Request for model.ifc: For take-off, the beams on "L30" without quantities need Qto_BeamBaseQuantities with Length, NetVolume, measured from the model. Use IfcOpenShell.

First a look at what the model holds.

```python
import ifcopenshell
import ifcopenshell.util.element
import ifcopenshell.util.unit

model = ifcopenshell.open("model.ifc")
print(model.schema)
for unit_type in ("LENGTHUNIT", "AREAUNIT", "VOLUMEUNIT"):
    print(unit_type, ifcopenshell.util.unit.calculate_unit_scale(model, unit_type))
storey = next(s for s in model.by_type("IfcBuildingStorey") if s.Name == "L30")
beams = [e for e in ifcopenshell.util.element.get_decomposition(storey) if e.is_a("IfcBeam")]
for e in sorted(beams, key=lambda e: e.id()):
    print(e.id(), e.is_a(), e.Name, list(ifcopenshell.util.element.get_psets(e, qtos_only=True)), sep=" | ")
```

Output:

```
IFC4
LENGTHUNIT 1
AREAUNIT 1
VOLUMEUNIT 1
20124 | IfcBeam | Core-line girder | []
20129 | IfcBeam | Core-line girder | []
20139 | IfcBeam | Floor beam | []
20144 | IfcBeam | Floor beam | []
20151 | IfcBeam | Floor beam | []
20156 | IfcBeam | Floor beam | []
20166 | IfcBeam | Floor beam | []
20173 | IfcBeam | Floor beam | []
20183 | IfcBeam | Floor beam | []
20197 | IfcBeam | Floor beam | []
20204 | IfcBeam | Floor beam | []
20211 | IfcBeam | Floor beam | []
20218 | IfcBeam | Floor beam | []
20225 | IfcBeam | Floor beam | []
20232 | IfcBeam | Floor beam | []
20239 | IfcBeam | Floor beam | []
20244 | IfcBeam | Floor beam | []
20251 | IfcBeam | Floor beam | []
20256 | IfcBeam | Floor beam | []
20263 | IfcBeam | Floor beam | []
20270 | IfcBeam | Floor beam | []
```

```python
import ifcopenshell
import ifcopenshell.api.pset
import ifcopenshell.geom
import ifcopenshell.util.element
import ifcopenshell.util.shape
import ifcopenshell.util.unit

model = ifcopenshell.open("model.ifc")
unit_scale = ifcopenshell.util.unit.calculate_unit_scale(model)
volume_scale = ifcopenshell.util.unit.calculate_unit_scale(model, "VOLUMEUNIT")
settings = ifcopenshell.geom.settings()

storey = next(s for s in model.by_type("IfcBuildingStorey") if s.Name == "L30")
beams = [e for e in ifcopenshell.util.element.get_decomposition(storey) if e.is_a("IfcBeam")]

for e in sorted(beams, key=lambda e: e.id()):
    if ifcopenshell.util.element.get_psets(e, qtos_only=True, should_inherit=False):
        continue
    # Geometry comes back in metres, in the element's own axes.
    shape = ifcopenshell.geom.create_shape(settings, e)
    values = {
        "Length": ifcopenshell.util.shape.get_max_xyz(shape.geometry) / unit_scale,
        "NetVolume": ifcopenshell.util.shape.get_volume(shape.geometry) / volume_scale,
    }
    qto = ifcopenshell.api.pset.add_qto(model, product=e, name="Qto_BeamBaseQuantities")
    ifcopenshell.api.pset.edit_qto(model, qto=qto, properties=values)
    print(e.id(), {k: round(v, 3) for k, v in values.items()})

model.write("model_updated.ifc")
```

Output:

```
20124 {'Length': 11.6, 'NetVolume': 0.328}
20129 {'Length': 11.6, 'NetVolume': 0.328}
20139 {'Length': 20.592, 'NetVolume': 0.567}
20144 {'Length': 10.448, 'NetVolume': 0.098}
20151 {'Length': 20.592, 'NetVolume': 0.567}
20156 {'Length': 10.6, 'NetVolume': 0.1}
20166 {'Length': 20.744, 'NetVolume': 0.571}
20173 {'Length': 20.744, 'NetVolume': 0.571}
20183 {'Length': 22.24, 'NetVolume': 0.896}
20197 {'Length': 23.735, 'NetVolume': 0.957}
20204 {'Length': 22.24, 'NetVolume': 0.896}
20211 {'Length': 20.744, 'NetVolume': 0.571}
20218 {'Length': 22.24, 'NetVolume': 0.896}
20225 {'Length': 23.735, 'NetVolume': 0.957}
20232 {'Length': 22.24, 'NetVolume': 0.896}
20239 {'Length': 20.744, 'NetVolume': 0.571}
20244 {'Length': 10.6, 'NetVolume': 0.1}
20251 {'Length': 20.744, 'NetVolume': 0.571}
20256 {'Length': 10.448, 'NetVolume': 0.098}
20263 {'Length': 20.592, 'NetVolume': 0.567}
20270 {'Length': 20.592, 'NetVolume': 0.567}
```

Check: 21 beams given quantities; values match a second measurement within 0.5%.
